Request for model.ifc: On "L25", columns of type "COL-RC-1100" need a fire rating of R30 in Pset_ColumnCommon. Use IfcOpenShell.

First a look at what the model holds.

```python
import ifcopenshell
import ifcopenshell.util.element

model = ifcopenshell.open("model.ifc")
print(model.schema)
storey = next(s for s in model.by_type("IfcBuildingStorey") if s.Name == "L25")
columns = [e for e in ifcopenshell.util.element.get_decomposition(storey) if e.is_a("IfcColumn")]
seen = {}
for e in columns:
    element_type = ifcopenshell.util.element.get_type(e)
    key = (element_type.Name if element_type != e and element_type else None, ifcopenshell.util.element.get_pset(e, "Pset_ColumnCommon", "FireRating"))
    seen[key] = seen.get(key, 0) + 1
for (name, value), count in sorted(seen.items(), key=str):
    print(count, "x", name, "|", value)
```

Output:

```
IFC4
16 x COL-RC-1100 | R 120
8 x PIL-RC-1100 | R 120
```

```python
import ifcopenshell
import ifcopenshell.api.pset
import ifcopenshell.util.element

model = ifcopenshell.open("model.ifc")

storey = next(s for s in model.by_type("IfcBuildingStorey") if s.Name == "L25")
columns = [e for e in ifcopenshell.util.element.get_decomposition(storey) if e.is_a("IfcColumn")]

count = 0
for e in columns:
    element_type = ifcopenshell.util.element.get_type(e)
    if element_type in (None, e) or element_type.Name != "COL-RC-1100":
        continue
    # add_pset returns the element's existing set when there is one.
    pset = ifcopenshell.api.pset.add_pset(model, product=e, name="Pset_ColumnCommon")
    ifcopenshell.api.pset.edit_pset(model, pset=pset, properties={"FireRating": "R30"})
    count += 1

print(count, "columns updated")

model.write("model_rev.ifc")
```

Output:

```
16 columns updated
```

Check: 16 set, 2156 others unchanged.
